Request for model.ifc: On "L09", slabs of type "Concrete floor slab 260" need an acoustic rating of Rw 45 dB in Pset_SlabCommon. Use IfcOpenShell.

First a look at what the model holds.

```python
import ifcopenshell
import ifcopenshell.util.element

model = ifcopenshell.open("model.ifc")
print(model.schema)
storey = next(s for s in model.by_type("IfcBuildingStorey") if s.Name == "L09")
slabs = [e for e in ifcopenshell.util.element.get_decomposition(storey) if e.is_a("IfcSlab")]
seen = {}
for e in slabs:
    element_type = ifcopenshell.util.element.get_type(e)
    key = (element_type.Name if element_type != e and element_type else None, ifcopenshell.util.element.get_pset(e, "Pset_SlabCommon", "AcousticRating"))
    seen[key] = seen.get(key, 0) + 1
for (name, value), count in sorted(seen.items(), key=str):
    print(count, "x", name, "|", value)
```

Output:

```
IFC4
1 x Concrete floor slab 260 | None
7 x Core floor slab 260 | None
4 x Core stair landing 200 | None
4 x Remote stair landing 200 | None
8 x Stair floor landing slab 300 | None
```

```python
import ifcopenshell
import ifcopenshell.api.pset
import ifcopenshell.util.element

model = ifcopenshell.open("model.ifc")

storey = next(s for s in model.by_type("IfcBuildingStorey") if s.Name == "L09")
slabs = [e for e in ifcopenshell.util.element.get_decomposition(storey) if e.is_a("IfcSlab")]

count = 0
for e in slabs:
    element_type = ifcopenshell.util.element.get_type(e)
    if element_type in (None, e) or element_type.Name != "Concrete floor slab 260":
        continue
    found = ifcopenshell.util.element.get_pset(e, "Pset_SlabCommon", should_inherit=False)
    if found:
        pset = model.by_id(found["id"])
        if len(ifcopenshell.util.element.get_elements_by_pset(pset)) > 1:
            pset = ifcopenshell.api.pset.unshare_pset(model, products=[e], pset=pset)[0]
    else:
        pset = ifcopenshell.api.pset.add_pset(model, product=e, name="Pset_SlabCommon")
    ifcopenshell.api.pset.edit_pset(model, pset=pset, properties={"AcousticRating": "Rw 45 dB"})
    count += 1

print(count, "slabs updated")

model.write("model_edited.ifc")
```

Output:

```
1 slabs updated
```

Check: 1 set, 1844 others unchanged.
